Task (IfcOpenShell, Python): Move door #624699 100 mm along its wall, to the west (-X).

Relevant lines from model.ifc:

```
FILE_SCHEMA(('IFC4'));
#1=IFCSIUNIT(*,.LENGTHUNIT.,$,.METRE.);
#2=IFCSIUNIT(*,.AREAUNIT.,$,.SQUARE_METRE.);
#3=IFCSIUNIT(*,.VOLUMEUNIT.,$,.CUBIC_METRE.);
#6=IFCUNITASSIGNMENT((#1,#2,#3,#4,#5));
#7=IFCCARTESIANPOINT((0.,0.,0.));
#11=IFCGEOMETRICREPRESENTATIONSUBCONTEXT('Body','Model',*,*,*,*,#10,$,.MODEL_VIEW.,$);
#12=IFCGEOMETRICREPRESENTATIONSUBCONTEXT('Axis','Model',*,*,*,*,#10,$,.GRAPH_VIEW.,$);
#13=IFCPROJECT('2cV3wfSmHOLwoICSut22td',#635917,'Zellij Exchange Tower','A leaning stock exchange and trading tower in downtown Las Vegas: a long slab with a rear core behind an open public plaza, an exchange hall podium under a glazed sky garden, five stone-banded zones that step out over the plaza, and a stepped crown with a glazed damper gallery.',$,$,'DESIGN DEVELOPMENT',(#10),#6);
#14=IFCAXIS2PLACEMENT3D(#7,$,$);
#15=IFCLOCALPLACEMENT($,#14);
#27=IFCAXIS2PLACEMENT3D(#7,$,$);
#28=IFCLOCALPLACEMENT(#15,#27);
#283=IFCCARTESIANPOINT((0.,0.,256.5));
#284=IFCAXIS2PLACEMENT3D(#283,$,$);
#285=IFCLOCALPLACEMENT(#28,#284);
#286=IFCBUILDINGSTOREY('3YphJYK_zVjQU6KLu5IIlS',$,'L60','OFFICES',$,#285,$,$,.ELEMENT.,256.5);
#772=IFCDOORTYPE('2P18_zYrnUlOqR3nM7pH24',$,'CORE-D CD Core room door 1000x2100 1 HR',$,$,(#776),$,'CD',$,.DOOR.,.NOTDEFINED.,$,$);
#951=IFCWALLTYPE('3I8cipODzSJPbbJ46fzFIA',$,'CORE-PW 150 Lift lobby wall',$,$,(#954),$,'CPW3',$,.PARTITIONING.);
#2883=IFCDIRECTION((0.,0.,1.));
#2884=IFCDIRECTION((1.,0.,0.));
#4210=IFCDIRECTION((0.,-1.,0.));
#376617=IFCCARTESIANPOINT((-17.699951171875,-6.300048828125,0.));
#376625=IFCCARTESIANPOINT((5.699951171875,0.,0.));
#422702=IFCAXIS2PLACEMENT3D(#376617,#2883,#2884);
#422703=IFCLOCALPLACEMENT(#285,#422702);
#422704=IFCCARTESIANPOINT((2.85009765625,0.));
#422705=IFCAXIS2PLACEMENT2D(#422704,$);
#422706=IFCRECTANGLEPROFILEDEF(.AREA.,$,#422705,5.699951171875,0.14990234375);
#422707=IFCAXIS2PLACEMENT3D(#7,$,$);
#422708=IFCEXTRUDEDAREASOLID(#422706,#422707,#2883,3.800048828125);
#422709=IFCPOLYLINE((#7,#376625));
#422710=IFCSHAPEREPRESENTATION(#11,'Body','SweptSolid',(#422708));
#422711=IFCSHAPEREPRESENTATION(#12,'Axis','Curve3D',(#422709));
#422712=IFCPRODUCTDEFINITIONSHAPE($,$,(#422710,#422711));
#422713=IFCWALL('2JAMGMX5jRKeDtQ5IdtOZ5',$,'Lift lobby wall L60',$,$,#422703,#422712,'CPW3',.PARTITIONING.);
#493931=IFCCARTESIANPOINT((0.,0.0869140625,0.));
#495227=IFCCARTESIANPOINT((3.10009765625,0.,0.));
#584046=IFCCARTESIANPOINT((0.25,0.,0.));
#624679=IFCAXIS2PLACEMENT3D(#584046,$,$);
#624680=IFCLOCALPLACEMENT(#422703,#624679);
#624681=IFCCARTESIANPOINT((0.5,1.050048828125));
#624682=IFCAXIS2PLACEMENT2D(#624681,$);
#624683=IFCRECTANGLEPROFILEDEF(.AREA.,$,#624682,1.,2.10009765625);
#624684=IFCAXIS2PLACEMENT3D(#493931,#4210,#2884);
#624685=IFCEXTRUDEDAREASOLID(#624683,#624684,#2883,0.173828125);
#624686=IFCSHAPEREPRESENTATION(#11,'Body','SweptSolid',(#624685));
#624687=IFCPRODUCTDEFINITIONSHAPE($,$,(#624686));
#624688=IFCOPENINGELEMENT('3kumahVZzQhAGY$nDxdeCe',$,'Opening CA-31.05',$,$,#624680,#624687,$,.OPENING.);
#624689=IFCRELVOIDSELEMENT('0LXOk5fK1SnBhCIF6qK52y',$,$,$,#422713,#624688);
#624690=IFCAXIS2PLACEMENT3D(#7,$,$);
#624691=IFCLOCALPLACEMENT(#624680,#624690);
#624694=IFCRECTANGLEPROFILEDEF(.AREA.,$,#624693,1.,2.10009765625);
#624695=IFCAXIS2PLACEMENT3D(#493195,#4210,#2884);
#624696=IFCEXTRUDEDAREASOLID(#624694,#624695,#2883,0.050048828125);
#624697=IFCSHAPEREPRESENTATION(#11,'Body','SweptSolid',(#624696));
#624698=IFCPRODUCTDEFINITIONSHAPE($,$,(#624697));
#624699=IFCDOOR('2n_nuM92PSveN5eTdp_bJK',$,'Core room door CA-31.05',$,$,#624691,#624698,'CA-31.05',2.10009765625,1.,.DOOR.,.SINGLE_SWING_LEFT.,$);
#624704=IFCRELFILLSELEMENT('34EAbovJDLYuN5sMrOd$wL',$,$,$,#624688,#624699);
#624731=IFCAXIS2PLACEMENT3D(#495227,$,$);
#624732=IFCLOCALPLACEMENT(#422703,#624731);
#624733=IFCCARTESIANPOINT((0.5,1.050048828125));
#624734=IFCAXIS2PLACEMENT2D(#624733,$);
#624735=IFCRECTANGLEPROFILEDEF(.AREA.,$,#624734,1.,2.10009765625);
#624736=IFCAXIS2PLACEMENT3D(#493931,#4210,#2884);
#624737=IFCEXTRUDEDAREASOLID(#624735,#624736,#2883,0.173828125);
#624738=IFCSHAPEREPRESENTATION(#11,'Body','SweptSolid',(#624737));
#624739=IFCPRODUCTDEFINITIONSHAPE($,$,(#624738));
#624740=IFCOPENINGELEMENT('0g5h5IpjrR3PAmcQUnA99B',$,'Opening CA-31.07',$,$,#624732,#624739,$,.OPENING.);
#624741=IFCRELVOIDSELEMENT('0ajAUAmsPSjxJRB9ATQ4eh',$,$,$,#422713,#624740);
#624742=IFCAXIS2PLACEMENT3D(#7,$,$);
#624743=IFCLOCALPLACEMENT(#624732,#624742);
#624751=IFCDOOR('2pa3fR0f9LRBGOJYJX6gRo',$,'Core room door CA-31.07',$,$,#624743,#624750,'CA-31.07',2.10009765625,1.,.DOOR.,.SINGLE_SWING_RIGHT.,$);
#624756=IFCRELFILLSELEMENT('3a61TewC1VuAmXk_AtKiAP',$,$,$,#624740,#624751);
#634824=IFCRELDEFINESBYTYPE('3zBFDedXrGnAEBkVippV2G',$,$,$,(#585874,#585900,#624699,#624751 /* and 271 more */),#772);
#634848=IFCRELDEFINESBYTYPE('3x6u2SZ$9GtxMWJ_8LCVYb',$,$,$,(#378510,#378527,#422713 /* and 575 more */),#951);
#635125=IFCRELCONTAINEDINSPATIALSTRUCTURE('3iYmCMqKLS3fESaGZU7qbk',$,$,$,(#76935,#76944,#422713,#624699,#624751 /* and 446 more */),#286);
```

```python
import ifcopenshell
import ifcopenshell.api.geometry
import ifcopenshell.util.placement
import ifcopenshell.util.unit

model = ifcopenshell.open("model.ifc")
unit_scale = ifcopenshell.util.unit.calculate_unit_scale(model)

door = model.by_id(624699)
opening = door.FillsVoids[0].RelatingOpeningElement
wall = opening.VoidsElements[0].RelatingBuildingElement

wall_matrix = ifcopenshell.util.placement.get_local_placement(wall.ObjectPlacement)
shift = wall_matrix[:3, 0] * -0.1 / unit_scale
before = ifcopenshell.util.placement.get_local_placement(door.ObjectPlacement)[:3, 3].copy()

# The door is placed relative to its opening, so it follows when the opening moves.
matrix = ifcopenshell.util.placement.get_local_placement(opening.ObjectPlacement)
matrix[:3, 3] += shift
ifcopenshell.api.geometry.edit_object_placement(
    model, product=opening, matrix=matrix, is_si=False, should_transform_children=True
)

after = ifcopenshell.util.placement.get_local_placement(door.ObjectPlacement)[:3, 3]
print("door moved by", (after - before).round(3) + 0.0)

model.write("model_v2.ifc")
```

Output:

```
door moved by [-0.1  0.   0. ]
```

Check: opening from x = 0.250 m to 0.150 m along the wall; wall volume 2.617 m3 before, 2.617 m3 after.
